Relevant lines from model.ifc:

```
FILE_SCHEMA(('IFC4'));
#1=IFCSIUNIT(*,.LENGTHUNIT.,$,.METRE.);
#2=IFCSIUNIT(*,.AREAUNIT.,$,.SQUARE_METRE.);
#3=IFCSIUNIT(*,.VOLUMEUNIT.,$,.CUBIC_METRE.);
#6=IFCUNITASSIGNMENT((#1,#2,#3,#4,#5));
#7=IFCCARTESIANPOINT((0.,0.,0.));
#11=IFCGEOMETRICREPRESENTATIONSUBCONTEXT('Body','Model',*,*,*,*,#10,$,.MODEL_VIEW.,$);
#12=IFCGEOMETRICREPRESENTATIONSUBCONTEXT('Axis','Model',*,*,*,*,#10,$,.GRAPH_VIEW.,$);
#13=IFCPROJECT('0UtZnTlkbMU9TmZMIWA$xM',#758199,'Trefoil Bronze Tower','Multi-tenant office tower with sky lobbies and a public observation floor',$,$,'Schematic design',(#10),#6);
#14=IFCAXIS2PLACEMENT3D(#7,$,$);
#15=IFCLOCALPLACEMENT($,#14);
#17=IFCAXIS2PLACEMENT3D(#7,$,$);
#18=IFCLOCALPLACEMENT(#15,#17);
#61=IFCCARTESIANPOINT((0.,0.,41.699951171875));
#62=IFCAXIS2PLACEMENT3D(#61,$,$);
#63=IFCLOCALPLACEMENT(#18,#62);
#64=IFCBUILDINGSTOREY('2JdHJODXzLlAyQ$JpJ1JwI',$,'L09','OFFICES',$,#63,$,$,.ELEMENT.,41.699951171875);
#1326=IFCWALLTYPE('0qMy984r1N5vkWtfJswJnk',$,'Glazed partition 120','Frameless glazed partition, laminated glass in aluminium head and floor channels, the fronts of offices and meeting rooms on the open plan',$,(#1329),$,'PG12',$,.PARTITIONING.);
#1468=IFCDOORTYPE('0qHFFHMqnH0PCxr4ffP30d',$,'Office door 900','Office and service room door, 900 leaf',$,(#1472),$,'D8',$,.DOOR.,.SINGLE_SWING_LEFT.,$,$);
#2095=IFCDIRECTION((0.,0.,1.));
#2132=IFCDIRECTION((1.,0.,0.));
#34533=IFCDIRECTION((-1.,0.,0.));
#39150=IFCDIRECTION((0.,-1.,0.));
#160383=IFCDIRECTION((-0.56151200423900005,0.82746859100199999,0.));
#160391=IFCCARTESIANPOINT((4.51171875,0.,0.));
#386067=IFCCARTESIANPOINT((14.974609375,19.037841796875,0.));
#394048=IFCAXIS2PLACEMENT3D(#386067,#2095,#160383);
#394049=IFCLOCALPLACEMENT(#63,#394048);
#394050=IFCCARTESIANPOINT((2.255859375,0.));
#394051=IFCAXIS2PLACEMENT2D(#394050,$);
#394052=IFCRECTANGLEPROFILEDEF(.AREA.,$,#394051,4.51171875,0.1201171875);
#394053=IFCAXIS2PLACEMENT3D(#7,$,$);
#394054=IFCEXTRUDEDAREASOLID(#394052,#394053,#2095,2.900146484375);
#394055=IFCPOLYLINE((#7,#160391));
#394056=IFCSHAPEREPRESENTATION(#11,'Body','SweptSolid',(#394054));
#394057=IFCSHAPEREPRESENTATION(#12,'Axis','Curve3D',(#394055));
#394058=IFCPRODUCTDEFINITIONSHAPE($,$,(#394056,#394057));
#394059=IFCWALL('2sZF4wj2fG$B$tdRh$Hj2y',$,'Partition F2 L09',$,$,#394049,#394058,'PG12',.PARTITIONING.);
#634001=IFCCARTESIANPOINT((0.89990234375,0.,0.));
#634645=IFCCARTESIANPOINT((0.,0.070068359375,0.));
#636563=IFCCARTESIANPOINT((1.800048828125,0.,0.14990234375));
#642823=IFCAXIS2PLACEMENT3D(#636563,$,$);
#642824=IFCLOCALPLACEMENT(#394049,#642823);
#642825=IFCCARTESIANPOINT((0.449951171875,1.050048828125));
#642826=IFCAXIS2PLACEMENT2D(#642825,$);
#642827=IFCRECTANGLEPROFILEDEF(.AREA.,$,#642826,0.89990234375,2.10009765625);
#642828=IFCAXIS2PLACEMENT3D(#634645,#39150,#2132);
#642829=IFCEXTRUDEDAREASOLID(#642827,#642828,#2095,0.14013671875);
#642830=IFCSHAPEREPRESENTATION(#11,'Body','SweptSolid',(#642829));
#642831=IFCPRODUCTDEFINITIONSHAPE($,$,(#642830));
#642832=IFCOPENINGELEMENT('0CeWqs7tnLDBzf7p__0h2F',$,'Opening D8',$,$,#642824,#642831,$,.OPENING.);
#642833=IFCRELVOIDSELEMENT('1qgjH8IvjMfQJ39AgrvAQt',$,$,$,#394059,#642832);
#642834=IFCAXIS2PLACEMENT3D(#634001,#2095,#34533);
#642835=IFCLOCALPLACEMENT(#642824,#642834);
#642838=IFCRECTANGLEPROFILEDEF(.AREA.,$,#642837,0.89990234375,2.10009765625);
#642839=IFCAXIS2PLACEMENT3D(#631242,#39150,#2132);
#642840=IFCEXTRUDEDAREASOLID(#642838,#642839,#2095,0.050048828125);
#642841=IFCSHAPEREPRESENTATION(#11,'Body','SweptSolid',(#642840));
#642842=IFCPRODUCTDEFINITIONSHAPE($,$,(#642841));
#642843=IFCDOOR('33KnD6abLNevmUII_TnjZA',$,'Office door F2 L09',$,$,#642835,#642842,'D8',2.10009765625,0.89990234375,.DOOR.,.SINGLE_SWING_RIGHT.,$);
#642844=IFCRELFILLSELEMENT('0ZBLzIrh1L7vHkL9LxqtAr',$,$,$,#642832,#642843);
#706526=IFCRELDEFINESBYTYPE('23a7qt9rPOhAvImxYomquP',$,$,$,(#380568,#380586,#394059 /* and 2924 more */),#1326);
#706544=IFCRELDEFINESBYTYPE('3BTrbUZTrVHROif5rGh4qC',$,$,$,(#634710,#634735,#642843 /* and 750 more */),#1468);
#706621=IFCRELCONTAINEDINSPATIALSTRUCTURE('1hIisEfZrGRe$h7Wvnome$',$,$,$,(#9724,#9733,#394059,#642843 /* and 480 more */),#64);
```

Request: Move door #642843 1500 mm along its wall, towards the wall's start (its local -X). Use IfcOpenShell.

```python
import ifcopenshell
import ifcopenshell.api.geometry
import ifcopenshell.util.placement
import ifcopenshell.util.unit

model = ifcopenshell.open("model.ifc")
unit_scale = ifcopenshell.util.unit.calculate_unit_scale(model)

door = model.by_guid("33KnD6abLNevmUII_TnjZA")
opening = door.FillsVoids[0].RelatingOpeningElement
wall = opening.VoidsElements[0].RelatingBuildingElement

wall_matrix = ifcopenshell.util.placement.get_local_placement(wall.ObjectPlacement)
shift = wall_matrix[:3, 0] * -1.5 / unit_scale
before = ifcopenshell.util.placement.get_local_placement(door.ObjectPlacement)[:3, 3].copy()

# The door is placed relative to its opening, so it follows when the opening moves.
matrix = ifcopenshell.util.placement.get_local_placement(opening.ObjectPlacement)
matrix[:3, 3] += shift
ifcopenshell.api.geometry.edit_object_placement(
    model, product=opening, matrix=matrix, is_si=False, should_transform_children=True
)

after = ifcopenshell.util.placement.get_local_placement(door.ObjectPlacement)[:3, 3]
print("door moved by", (after - before).round(3) + 0.0)

model.write("model-out.ifc")
```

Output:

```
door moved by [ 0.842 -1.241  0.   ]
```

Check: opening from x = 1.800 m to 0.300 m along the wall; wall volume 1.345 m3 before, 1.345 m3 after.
